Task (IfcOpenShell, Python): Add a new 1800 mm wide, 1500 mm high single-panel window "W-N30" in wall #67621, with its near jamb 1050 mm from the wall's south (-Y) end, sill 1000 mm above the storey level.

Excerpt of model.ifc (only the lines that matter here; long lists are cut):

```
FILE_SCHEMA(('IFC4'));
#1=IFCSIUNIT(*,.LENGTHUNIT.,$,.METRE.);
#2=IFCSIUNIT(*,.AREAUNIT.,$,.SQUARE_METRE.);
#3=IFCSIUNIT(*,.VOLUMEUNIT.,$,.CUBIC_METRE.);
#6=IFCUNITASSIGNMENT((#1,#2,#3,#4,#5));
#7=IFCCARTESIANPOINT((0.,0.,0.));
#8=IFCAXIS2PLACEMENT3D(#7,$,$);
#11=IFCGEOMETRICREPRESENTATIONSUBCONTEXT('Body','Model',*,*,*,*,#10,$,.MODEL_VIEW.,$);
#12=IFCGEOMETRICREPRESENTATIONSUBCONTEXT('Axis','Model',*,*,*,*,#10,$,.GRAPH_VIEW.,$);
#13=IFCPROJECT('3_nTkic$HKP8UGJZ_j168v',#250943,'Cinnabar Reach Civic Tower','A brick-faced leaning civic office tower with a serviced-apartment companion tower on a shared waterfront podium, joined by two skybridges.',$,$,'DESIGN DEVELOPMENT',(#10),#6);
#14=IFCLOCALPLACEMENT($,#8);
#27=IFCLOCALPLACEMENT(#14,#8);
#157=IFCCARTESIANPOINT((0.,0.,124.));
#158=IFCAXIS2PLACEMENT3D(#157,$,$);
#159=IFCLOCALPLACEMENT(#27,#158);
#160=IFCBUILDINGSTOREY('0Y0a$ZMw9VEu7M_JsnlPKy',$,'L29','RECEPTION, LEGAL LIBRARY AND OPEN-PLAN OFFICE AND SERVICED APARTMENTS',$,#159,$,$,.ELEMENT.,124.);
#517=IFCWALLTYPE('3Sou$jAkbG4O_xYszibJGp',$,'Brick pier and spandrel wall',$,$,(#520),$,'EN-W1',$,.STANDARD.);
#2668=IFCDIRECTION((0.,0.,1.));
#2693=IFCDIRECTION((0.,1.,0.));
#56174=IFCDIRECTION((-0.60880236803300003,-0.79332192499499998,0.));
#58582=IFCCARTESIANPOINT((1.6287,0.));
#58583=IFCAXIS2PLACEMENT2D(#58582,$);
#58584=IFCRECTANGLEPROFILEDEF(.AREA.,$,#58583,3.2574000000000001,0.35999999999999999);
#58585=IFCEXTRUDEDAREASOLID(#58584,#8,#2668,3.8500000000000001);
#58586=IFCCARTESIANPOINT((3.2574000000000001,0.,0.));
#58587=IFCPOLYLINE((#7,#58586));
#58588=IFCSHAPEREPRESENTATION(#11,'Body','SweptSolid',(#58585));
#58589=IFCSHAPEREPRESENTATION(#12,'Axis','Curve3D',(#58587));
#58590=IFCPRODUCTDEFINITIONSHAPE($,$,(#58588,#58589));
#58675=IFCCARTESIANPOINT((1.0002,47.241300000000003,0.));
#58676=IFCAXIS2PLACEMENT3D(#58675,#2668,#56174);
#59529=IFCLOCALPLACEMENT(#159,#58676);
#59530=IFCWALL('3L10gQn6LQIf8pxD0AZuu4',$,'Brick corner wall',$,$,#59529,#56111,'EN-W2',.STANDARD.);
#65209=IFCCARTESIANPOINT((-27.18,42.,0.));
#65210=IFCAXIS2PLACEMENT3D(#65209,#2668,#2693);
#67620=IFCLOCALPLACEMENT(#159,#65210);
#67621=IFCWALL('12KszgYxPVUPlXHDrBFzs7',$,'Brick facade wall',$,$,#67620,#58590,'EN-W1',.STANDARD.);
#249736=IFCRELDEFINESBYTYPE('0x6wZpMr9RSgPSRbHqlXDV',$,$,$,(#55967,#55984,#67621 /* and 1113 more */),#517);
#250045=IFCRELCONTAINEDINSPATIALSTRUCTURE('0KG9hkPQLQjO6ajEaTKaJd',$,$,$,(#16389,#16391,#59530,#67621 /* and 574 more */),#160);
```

```python
import numpy as np
import ifcopenshell
import ifcopenshell.api.feature
import ifcopenshell.api.geometry
import ifcopenshell.api.root
import ifcopenshell.api.spatial
import ifcopenshell.geom
import ifcopenshell.util.element
import ifcopenshell.util.placement
import ifcopenshell.util.representation
import ifcopenshell.util.shape
import ifcopenshell.util.unit

model = ifcopenshell.open("model.ifc")
unit_scale = ifcopenshell.util.unit.calculate_unit_scale(model)
settings = ifcopenshell.geom.settings()


def volume(element):
    """Net volume in cubic metres, openings subtracted."""
    shape = ifcopenshell.geom.create_shape(settings, element)
    return ifcopenshell.util.shape.get_volume(shape.geometry)


wall = model.by_id(67621)
storey = ifcopenshell.util.element.get_container(wall, ifc_class="IfcBuildingStorey")
context = ifcopenshell.util.representation.get_context(model, "Model", "Body", "MODEL_VIEW")
before = volume(wall)

width, height, from_end, sill = 1.8, 1.5, 1.05, 1  # metres

# The wall runs along its own X axis, and the end named is its -X end.
wall_shape = ifcopenshell.geom.create_shape(settings, wall)
x, y, z = ifcopenshell.util.shape.get_vertices(wall_shape.geometry).T
start = x.min() + from_end
face, thickness = float(y.min()), float(y.max() - y.min())
wall_matrix = ifcopenshell.util.placement.get_local_placement(wall.ObjectPlacement)
level = ifcopenshell.util.placement.get_local_placement(storey.ObjectPlacement)[2, 3]


def in_wall(x, y):
    """Placement at x, y metres in the wall's axes, at sill height."""
    matrix = wall_matrix.copy()
    matrix[:, 3] = wall_matrix @ np.array([x / unit_scale, y / unit_scale, 0.0, 1.0])
    matrix[2, 3] = level + sill / unit_scale
    return matrix


# Opening: a box that overshoots both wall faces by 50 mm.
opening = ifcopenshell.api.root.create_entity(model, ifc_class="IfcOpeningElement", predefined_type="OPENING")
box = ifcopenshell.api.geometry.add_wall_representation(
    model, context=context, length=width, height=height, thickness=thickness + 0.1
)
ifcopenshell.api.geometry.assign_representation(model, product=opening, representation=box)
ifcopenshell.api.geometry.edit_object_placement(model, product=opening, matrix=in_wall(start, face - 0.05), is_si=False)
ifcopenshell.api.feature.add_feature(model, feature=opening, element=wall)

window = ifcopenshell.api.root.create_entity(model, ifc_class="IfcWindow", name="W-N30", predefined_type="WINDOW")
window.OverallWidth, window.OverallHeight = width / unit_scale, height / unit_scale
window.PartitioningType = "SINGLE_PANEL"
body = ifcopenshell.api.geometry.add_window_representation(
    model,
    context=context,
    overall_width=window.OverallWidth,
    overall_height=window.OverallHeight,
    partition_type="SINGLE_PANEL",
)
ifcopenshell.api.geometry.assign_representation(model, product=window, representation=body)
ifcopenshell.api.spatial.assign_container(model, products=[window], relating_structure=storey)
ifcopenshell.api.feature.add_filling(model, opening=opening, element=window)

# Centre the window in the wall's thickness.
ifcopenshell.api.geometry.edit_object_placement(model, product=window, matrix=in_wall(start, face), is_si=False)
window_shape = ifcopenshell.geom.create_shape(settings, window)
depth = ifcopenshell.util.shape.get_vertices(window_shape.geometry)[:, 1]
offset = face + thickness / 2 - (depth.min() + depth.max()) / 2
ifcopenshell.api.geometry.edit_object_placement(model, product=window, matrix=in_wall(start, offset), is_si=False)

after = volume(wall)

print(f"wall volume {before:.3f} -> {after:.3f} m3")

model.write("model_v2.ifc")
```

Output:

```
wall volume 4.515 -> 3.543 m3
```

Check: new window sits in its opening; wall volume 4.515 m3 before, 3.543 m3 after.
